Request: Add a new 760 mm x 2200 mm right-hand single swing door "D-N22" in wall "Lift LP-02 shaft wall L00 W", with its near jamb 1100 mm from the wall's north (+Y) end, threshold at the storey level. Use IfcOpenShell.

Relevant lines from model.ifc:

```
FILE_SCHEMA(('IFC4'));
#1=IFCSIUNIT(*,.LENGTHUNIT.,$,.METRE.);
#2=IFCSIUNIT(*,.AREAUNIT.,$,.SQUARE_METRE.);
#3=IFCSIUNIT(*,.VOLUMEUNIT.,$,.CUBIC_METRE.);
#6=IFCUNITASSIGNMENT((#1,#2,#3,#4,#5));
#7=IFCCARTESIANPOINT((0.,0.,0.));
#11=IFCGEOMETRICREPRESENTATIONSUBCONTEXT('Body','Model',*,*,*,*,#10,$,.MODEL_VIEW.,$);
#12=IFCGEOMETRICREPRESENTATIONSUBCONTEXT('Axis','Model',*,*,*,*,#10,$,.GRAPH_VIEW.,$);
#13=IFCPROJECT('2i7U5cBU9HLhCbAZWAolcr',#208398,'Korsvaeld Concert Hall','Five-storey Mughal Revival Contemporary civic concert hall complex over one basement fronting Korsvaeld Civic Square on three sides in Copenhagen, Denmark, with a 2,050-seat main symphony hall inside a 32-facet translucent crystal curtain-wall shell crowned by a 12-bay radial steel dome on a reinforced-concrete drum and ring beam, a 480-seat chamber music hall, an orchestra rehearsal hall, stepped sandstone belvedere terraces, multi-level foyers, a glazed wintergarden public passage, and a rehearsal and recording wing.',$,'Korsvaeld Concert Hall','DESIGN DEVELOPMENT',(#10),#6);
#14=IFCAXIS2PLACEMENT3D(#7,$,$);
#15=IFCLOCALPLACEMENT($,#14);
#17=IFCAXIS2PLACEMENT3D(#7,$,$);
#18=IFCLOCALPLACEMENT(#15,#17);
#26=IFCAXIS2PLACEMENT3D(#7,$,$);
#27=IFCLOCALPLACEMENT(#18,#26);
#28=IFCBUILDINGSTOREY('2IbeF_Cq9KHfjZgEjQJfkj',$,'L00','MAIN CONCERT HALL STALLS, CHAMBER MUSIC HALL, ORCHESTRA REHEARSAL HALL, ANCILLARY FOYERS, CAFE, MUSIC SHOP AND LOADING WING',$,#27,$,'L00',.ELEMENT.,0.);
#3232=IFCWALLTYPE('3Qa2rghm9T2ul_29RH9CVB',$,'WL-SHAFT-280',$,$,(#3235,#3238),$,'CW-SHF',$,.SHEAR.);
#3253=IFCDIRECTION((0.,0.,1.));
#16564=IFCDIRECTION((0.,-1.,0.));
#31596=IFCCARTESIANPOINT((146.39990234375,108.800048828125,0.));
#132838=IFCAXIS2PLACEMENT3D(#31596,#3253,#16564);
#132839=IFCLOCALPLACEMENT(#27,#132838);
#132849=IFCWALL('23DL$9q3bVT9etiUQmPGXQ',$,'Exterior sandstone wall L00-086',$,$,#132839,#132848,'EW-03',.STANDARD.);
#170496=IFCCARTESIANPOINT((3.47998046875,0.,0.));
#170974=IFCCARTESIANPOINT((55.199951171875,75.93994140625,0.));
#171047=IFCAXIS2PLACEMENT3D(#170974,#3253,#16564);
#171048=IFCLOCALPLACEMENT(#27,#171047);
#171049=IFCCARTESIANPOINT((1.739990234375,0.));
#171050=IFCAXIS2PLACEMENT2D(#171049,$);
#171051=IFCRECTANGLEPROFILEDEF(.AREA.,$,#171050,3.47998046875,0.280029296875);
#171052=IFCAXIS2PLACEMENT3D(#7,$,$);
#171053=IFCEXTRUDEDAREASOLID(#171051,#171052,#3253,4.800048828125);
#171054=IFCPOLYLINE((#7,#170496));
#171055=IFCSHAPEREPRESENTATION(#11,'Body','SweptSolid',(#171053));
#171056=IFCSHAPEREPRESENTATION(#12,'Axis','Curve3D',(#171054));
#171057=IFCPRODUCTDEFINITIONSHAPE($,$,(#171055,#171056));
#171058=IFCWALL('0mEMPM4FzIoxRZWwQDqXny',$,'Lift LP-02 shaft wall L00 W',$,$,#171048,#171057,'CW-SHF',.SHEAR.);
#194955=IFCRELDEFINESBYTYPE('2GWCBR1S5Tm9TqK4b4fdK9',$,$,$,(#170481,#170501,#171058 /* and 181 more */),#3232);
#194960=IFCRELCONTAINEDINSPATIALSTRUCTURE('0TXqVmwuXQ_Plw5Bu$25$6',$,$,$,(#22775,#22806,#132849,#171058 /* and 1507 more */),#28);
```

```python
import numpy as np
import ifcopenshell
import ifcopenshell.api.feature
import ifcopenshell.api.geometry
import ifcopenshell.api.root
import ifcopenshell.api.spatial
import ifcopenshell.geom
import ifcopenshell.util.element
import ifcopenshell.util.placement
import ifcopenshell.util.representation
import ifcopenshell.util.shape
import ifcopenshell.util.unit

model = ifcopenshell.open("model.ifc")
unit_scale = ifcopenshell.util.unit.calculate_unit_scale(model)
settings = ifcopenshell.geom.settings()


def volume(element):
    """Net volume in cubic metres, openings subtracted."""
    shape = ifcopenshell.geom.create_shape(settings, element)
    return ifcopenshell.util.shape.get_volume(shape.geometry)


wall = model.by_guid("0mEMPM4FzIoxRZWwQDqXny")
storey = ifcopenshell.util.element.get_container(wall, ifc_class="IfcBuildingStorey")
context = ifcopenshell.util.representation.get_context(model, "Model", "Body", "MODEL_VIEW")
before = volume(wall)

width, height, from_end, sill = 0.76, 2.2, 1.1, 0.0  # metres

# The wall runs along its own X axis, and the end named is its -X end.
wall_shape = ifcopenshell.geom.create_shape(settings, wall)
x, y, z = ifcopenshell.util.shape.get_vertices(wall_shape.geometry).T
start = x.min() + from_end
face, thickness = float(y.min()), float(y.max() - y.min())
wall_matrix = ifcopenshell.util.placement.get_local_placement(wall.ObjectPlacement)
level = ifcopenshell.util.placement.get_local_placement(storey.ObjectPlacement)[2, 3]


def in_wall(x, y):
    """Placement at x, y metres in the wall's axes, at sill height."""
    matrix = wall_matrix.copy()
    matrix[:, 3] = wall_matrix @ np.array([x / unit_scale, y / unit_scale, 0.0, 1.0])
    matrix[2, 3] = level + sill / unit_scale
    return matrix


# Opening: a box that overshoots both wall faces by 50 mm.
opening = ifcopenshell.api.root.create_entity(model, ifc_class="IfcOpeningElement", predefined_type="OPENING")
box = ifcopenshell.api.geometry.add_wall_representation(
    model, context=context, length=width, height=height, thickness=thickness + 0.1
)
ifcopenshell.api.geometry.assign_representation(model, product=opening, representation=box)
ifcopenshell.api.geometry.edit_object_placement(model, product=opening, matrix=in_wall(start, face - 0.05), is_si=False)
ifcopenshell.api.feature.add_feature(model, feature=opening, element=wall)

door = ifcopenshell.api.root.create_entity(model, ifc_class="IfcDoor", name="D-N22", predefined_type="DOOR")
door.OverallWidth, door.OverallHeight = width / unit_scale, height / unit_scale
door.OperationType = "SINGLE_SWING_RIGHT"
body = ifcopenshell.api.geometry.add_door_representation(
    model,
    context=context,
    overall_width=door.OverallWidth,
    overall_height=door.OverallHeight,
    operation_type="SINGLE_SWING_RIGHT",
    lining_properties={"LiningDepth": thickness / unit_scale, "ThresholdDepth": thickness / unit_scale},
)
ifcopenshell.api.geometry.assign_representation(model, product=door, representation=body)
ifcopenshell.api.spatial.assign_container(model, products=[door], relating_structure=storey)
ifcopenshell.api.feature.add_filling(model, opening=opening, element=door)

# The lining spans the wall, so the door starts at the wall face.
ifcopenshell.api.geometry.edit_object_placement(model, product=door, matrix=in_wall(start, face), is_si=False)

after = volume(wall)

print(f"wall volume {before:.3f} -> {after:.3f} m3")

model.write("model_edited.ifc")
```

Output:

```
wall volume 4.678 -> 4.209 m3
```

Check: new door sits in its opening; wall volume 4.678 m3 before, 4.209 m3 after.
